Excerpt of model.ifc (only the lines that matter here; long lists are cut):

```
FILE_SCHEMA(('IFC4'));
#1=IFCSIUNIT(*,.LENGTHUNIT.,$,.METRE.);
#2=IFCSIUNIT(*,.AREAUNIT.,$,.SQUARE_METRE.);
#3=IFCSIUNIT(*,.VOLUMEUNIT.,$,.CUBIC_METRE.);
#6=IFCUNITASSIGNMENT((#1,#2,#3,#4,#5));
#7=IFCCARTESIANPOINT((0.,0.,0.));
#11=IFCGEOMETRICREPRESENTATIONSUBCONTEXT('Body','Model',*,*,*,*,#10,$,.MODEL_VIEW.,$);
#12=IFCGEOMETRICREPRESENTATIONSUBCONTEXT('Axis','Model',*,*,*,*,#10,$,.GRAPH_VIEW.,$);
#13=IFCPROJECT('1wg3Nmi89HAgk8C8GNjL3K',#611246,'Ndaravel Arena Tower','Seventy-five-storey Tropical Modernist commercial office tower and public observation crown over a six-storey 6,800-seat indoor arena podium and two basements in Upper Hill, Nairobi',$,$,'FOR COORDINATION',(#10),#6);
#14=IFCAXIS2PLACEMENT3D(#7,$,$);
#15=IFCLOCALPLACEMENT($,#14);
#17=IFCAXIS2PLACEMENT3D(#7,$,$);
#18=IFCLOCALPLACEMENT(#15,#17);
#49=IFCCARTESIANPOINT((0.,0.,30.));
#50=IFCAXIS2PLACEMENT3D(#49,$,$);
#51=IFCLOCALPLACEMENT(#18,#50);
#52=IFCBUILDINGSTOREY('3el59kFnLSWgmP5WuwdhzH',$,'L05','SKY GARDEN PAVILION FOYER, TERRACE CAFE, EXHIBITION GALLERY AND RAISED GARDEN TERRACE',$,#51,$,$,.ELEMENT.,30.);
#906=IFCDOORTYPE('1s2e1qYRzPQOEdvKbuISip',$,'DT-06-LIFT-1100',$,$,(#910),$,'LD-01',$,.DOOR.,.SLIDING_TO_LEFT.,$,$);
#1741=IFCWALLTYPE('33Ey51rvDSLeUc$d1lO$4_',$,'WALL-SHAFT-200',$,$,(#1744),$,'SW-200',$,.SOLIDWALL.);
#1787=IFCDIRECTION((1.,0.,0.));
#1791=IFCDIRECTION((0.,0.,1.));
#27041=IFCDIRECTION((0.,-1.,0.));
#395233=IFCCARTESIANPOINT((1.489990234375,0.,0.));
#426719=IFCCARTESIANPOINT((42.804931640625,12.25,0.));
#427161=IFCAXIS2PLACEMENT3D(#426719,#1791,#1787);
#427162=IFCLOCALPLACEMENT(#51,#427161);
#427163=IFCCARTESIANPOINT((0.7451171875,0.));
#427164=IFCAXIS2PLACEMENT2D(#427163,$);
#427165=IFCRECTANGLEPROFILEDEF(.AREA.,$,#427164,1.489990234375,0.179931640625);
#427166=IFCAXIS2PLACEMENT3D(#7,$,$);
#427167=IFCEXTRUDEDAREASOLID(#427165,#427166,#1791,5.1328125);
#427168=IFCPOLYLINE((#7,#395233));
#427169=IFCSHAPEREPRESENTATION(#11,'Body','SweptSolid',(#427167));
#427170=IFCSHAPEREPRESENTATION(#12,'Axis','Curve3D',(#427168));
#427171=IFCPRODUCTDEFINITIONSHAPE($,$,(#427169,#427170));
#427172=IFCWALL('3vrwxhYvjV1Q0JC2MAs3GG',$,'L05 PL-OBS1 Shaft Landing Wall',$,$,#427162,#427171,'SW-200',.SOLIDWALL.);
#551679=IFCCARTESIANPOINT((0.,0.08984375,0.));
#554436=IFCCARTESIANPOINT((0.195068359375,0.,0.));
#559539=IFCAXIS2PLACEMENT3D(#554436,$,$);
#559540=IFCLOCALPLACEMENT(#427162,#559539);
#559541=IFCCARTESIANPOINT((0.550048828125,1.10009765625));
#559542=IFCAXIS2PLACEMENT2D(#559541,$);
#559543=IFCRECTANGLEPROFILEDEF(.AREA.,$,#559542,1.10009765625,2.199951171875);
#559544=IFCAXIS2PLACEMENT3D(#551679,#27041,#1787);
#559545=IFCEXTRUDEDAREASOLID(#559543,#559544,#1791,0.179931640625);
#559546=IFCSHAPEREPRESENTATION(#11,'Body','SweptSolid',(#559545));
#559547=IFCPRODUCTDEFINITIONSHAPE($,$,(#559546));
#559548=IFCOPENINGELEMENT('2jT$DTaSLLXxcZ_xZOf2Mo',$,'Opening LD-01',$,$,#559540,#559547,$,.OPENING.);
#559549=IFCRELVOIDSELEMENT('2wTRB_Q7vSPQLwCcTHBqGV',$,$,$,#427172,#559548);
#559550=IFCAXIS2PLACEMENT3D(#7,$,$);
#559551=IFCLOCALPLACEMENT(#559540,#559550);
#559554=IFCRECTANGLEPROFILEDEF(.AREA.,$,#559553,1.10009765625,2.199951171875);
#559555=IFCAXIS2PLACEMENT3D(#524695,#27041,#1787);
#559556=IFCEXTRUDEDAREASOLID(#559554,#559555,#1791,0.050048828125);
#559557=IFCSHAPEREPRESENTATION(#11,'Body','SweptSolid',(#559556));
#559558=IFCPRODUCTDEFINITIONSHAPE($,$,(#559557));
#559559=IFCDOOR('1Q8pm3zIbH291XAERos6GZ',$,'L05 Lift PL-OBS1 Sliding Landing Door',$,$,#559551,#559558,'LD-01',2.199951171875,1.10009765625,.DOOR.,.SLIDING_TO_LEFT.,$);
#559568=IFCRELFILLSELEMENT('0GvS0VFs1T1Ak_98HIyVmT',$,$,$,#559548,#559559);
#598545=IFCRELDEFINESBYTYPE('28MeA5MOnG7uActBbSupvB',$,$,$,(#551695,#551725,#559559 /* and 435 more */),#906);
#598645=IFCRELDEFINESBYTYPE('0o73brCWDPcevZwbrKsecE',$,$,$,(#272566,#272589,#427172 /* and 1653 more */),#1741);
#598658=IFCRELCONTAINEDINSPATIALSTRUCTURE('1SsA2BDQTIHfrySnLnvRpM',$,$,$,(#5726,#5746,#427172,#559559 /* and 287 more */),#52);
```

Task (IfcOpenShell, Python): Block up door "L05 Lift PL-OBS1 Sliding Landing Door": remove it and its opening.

```python
import ifcopenshell
import ifcopenshell.api.feature
import ifcopenshell.api.root
import ifcopenshell.geom
import ifcopenshell.util.shape

model = ifcopenshell.open("model.ifc")
settings = ifcopenshell.geom.settings()


def volume(element):
    """Net volume in cubic metres, openings subtracted."""
    shape = ifcopenshell.geom.create_shape(settings, element)
    return ifcopenshell.util.shape.get_volume(shape.geometry)


door = model.by_id(559559)
opening = door.FillsVoids[0].RelatingOpeningElement
wall = opening.VoidsElements[0].RelatingBuildingElement
before = volume(wall)

ifcopenshell.api.root.remove_product(model, product=door)
ifcopenshell.api.feature.remove_feature(model, feature=opening)

after = volume(wall)

print(f"wall volume {before:.3f} -> {after:.3f} m3")

model.write("model_v2.ifc")
```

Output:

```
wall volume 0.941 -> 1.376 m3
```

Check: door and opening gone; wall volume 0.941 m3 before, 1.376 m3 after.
